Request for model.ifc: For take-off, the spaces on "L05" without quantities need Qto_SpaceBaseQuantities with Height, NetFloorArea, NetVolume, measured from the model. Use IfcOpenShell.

First a look at what the model holds.

```python
import ifcopenshell
import ifcopenshell.util.element
import ifcopenshell.util.unit

model = ifcopenshell.open("model.ifc")
print(model.schema)
for unit_type in ("LENGTHUNIT", "AREAUNIT", "VOLUMEUNIT"):
    print(unit_type, ifcopenshell.util.unit.calculate_unit_scale(model, unit_type))
storey = next(s for s in model.by_type("IfcBuildingStorey") if s.Name == "L05")
spaces = [e for e in ifcopenshell.util.element.get_decomposition(storey) if e.is_a("IfcSpace")]
for e in sorted(spaces, key=lambda e: e.id()):
    print(e.id(), e.is_a(), e.Name, list(ifcopenshell.util.element.get_psets(e, qtos_only=True)), sep=" | ")
```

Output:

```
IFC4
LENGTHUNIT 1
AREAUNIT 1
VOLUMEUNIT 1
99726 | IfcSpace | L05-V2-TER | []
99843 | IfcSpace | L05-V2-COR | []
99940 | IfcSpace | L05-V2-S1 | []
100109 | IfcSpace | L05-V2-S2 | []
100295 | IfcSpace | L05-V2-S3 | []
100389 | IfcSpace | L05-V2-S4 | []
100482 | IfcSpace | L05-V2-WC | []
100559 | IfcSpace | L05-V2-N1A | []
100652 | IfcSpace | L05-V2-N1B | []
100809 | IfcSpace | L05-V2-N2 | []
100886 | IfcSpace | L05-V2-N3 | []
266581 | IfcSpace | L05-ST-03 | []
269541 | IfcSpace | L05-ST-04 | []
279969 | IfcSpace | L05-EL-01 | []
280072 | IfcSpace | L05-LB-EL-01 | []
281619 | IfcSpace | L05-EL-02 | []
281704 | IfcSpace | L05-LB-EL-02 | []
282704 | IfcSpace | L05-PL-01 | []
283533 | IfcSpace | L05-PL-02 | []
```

```python
import ifcopenshell
import ifcopenshell.api.pset
import ifcopenshell.geom
import ifcopenshell.util.element
import ifcopenshell.util.shape
import ifcopenshell.util.unit

model = ifcopenshell.open("model.ifc")
unit_scale = ifcopenshell.util.unit.calculate_unit_scale(model)
area_scale = ifcopenshell.util.unit.calculate_unit_scale(model, "AREAUNIT")
volume_scale = ifcopenshell.util.unit.calculate_unit_scale(model, "VOLUMEUNIT")
settings = ifcopenshell.geom.settings()

storey = next(s for s in model.by_type("IfcBuildingStorey") if s.Name == "L05")
spaces = [e for e in ifcopenshell.util.element.get_decomposition(storey) if e.is_a("IfcSpace")]

for e in sorted(spaces, key=lambda e: e.id()):
    if ifcopenshell.util.element.get_psets(e, qtos_only=True, should_inherit=False):
        continue
    # Geometry comes back in metres, in the element's own axes.
    shape = ifcopenshell.geom.create_shape(settings, e)
    values = {
        "Height": ifcopenshell.util.shape.get_z(shape.geometry) / unit_scale,
        "NetFloorArea": ifcopenshell.util.shape.get_footprint_area(shape.geometry) / area_scale,
        "NetVolume": ifcopenshell.util.shape.get_volume(shape.geometry) / volume_scale,
    }
    qto = ifcopenshell.api.pset.add_qto(model, product=e, name="Qto_SpaceBaseQuantities")
    ifcopenshell.api.pset.edit_qto(model, qto=qto, properties=values)
    print(e.id(), {k: round(v, 3) for k, v in values.items()})

model.write("model_edited.ifc")
```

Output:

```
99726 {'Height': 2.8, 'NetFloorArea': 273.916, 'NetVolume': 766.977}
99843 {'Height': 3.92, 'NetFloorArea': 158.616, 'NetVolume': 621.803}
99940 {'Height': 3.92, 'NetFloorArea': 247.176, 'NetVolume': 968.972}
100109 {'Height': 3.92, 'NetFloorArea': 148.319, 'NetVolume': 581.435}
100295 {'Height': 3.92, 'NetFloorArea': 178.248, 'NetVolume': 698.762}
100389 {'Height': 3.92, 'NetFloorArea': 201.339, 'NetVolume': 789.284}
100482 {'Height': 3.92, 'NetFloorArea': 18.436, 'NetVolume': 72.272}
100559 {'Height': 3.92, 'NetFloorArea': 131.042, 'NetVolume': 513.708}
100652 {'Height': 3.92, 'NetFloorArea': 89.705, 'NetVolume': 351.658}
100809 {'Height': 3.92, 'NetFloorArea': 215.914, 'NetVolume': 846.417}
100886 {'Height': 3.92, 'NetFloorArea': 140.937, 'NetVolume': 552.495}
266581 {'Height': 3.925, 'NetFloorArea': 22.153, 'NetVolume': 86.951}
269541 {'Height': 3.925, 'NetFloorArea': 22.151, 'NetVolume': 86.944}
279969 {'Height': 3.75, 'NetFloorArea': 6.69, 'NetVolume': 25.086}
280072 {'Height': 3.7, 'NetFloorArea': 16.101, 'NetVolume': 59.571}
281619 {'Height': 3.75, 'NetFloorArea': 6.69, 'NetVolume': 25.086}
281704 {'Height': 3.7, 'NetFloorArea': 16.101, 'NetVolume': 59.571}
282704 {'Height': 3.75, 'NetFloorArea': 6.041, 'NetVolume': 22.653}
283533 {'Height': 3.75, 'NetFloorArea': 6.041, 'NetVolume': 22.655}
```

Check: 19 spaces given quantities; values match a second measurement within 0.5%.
